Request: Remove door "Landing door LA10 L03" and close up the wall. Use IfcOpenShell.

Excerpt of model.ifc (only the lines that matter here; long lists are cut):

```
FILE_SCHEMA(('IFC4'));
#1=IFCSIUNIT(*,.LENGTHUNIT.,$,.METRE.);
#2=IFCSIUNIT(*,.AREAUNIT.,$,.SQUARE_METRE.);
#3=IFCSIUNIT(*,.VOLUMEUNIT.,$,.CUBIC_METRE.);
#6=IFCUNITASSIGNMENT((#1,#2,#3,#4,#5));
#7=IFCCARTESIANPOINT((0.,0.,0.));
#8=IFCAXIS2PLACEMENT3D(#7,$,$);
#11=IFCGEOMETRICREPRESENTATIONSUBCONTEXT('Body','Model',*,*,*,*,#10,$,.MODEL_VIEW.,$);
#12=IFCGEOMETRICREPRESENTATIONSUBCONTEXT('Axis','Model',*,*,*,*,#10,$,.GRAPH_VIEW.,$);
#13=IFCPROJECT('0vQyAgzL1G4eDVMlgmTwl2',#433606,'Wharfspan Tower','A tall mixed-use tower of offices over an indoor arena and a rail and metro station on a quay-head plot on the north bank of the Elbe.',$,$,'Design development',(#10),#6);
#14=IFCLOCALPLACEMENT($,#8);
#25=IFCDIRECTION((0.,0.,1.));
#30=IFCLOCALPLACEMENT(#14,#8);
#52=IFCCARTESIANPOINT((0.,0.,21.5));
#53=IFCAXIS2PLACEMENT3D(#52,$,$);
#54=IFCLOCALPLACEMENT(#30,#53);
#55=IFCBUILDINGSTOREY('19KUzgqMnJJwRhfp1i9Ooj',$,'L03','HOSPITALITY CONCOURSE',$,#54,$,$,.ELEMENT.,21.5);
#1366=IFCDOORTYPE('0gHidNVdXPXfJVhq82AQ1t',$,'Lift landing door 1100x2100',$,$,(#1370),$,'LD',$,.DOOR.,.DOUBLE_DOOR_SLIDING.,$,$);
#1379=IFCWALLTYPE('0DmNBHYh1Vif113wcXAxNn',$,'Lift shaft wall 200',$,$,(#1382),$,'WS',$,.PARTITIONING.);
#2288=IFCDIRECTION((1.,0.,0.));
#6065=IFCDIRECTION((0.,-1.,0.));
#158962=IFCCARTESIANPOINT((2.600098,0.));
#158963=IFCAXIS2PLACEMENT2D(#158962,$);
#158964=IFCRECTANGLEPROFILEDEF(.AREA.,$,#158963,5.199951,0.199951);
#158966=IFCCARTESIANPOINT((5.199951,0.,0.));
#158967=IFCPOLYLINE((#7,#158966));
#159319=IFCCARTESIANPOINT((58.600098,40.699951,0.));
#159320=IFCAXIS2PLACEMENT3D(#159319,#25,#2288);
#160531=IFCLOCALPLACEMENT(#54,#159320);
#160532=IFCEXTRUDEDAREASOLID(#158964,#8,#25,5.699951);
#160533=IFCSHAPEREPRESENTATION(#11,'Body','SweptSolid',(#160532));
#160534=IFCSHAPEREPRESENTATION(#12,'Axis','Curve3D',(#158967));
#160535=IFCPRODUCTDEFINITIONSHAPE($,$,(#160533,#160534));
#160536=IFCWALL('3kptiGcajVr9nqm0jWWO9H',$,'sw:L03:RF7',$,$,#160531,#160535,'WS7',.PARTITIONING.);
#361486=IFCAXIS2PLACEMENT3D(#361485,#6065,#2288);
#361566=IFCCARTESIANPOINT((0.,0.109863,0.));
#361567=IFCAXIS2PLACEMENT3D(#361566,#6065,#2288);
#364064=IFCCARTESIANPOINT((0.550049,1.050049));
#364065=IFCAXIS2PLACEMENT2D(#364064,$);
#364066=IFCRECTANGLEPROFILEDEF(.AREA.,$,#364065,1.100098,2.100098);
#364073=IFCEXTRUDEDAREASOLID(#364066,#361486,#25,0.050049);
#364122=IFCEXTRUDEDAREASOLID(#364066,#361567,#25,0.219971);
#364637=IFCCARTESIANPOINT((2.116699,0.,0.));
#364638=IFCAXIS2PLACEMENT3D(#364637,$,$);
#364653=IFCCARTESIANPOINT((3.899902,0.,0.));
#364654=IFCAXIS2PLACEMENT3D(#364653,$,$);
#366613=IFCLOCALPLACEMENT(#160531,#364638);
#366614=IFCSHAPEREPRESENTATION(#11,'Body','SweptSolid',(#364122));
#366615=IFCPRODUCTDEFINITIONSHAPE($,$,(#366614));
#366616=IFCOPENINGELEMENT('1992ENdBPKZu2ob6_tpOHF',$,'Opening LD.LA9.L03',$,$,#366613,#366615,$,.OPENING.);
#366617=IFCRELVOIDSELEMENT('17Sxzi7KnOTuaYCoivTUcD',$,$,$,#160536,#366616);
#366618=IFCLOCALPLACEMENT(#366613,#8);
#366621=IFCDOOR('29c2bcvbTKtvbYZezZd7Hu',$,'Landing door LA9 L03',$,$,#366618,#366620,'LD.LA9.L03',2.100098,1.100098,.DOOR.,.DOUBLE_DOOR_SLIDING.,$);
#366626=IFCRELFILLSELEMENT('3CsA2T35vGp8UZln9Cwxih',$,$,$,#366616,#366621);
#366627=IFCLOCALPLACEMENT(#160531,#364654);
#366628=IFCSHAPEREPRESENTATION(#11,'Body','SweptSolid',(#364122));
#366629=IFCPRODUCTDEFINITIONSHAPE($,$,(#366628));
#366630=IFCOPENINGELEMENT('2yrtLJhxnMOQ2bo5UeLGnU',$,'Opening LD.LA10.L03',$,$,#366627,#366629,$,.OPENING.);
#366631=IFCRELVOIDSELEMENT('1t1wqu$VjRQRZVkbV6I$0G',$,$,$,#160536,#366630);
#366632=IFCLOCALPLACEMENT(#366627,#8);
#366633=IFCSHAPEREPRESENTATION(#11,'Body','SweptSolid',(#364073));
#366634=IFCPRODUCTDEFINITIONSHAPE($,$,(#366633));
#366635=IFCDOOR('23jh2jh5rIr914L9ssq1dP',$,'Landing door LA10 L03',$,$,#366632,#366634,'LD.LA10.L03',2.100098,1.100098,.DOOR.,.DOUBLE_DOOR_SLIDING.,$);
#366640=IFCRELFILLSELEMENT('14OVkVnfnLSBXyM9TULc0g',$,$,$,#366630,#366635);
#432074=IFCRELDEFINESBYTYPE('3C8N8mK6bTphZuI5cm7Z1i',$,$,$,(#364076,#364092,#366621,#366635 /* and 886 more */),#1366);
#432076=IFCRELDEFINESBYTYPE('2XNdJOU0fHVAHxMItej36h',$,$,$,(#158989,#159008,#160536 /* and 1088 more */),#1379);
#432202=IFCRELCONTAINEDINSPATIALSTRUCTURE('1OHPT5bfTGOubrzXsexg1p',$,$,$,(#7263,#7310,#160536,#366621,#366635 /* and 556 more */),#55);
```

```python
import ifcopenshell
import ifcopenshell.api.feature
import ifcopenshell.api.root
import ifcopenshell.geom
import ifcopenshell.util.shape

model = ifcopenshell.open("model.ifc")
settings = ifcopenshell.geom.settings()


def volume(element):
    """Net volume in cubic metres, openings subtracted."""
    shape = ifcopenshell.geom.create_shape(settings, element)
    return ifcopenshell.util.shape.get_volume(shape.geometry)


door = model.by_guid("23jh2jh5rIr914L9ssq1dP")
opening = door.FillsVoids[0].RelatingOpeningElement
wall = opening.VoidsElements[0].RelatingBuildingElement
before = volume(wall)

ifcopenshell.api.root.remove_product(model, product=door)
ifcopenshell.api.feature.remove_feature(model, feature=opening)

after = volume(wall)

print(f"wall volume {before:.3f} -> {after:.3f} m3")

model.write("model_v2.ifc")
```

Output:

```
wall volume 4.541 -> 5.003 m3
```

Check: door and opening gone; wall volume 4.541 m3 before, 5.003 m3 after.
